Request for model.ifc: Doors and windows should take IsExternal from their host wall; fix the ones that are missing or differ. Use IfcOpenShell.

First a look at what the model holds.

```python
import ifcopenshell
import ifcopenshell.util.element

model = ifcopenshell.open("model.ifc")
print(model.schema)
seen = {}
for e in model.by_type("IfcDoor") + model.by_type("IfcWindow"):
    if not e.FillsVoids:
        continue
    host = e.FillsVoids[0].RelatingOpeningElement.VoidsElements[0].RelatingBuildingElement
    own = ifcopenshell.util.element.get_pset(e, f"Pset_{e.is_a()[3:].removesuffix('StandardCase')}Common", "IsExternal")
    wall = ifcopenshell.util.element.get_pset(host, "Pset_WallCommon", "IsExternal")
    seen[e.is_a(), own, wall] = seen.get((e.is_a(), own, wall), 0) + 1
for (cls, own, wall), count in sorted(seen.items(), key=str):
    print(count, cls, "IsExternal:", own, "| host wall:", wall)
```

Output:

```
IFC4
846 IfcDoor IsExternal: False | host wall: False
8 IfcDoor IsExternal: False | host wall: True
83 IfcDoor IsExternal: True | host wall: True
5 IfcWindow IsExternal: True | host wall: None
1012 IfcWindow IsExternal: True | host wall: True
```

```python
import ifcopenshell
import ifcopenshell.api.pset
import ifcopenshell.util.element

model = ifcopenshell.open("model.ifc")

count = 0
for ifc_class, pset_name in (("IfcDoor", "Pset_DoorCommon"), ("IfcWindow", "Pset_WindowCommon")):
    for e in model.by_type(ifc_class):
        if not e.FillsVoids:
            continue
        host = e.FillsVoids[0].RelatingOpeningElement.VoidsElements[0].RelatingBuildingElement
        external = ifcopenshell.util.element.get_pset(host, "Pset_WallCommon", "IsExternal")
        if external is None or ifcopenshell.util.element.get_pset(e, pset_name, "IsExternal") == external:
            continue
        pset = ifcopenshell.api.pset.add_pset(model, product=e, name=pset_name)
        ifcopenshell.api.pset.edit_pset(model, pset=pset, properties={"IsExternal": external})
        count += 1

print(count, "updated")

model.write("model_edited.ifc")
```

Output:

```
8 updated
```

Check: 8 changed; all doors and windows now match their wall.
